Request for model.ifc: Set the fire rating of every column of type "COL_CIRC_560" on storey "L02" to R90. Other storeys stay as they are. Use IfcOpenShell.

First a look at what the model holds.

```python
import ifcopenshell
import ifcopenshell.util.element

model = ifcopenshell.open("model.ifc")
print(model.schema)
storey = next(s for s in model.by_type("IfcBuildingStorey") if s.Name == "L02")
columns = [e for e in ifcopenshell.util.element.get_decomposition(storey) if e.is_a("IfcColumn")]
seen = {}
for e in columns:
    element_type = ifcopenshell.util.element.get_type(e)
    key = (element_type.Name if element_type != e and element_type else None, ifcopenshell.util.element.get_pset(e, "Pset_ColumnCommon", "FireRating"))
    seen[key] = seen.get(key, 0) + 1
for (name, value), count in sorted(seen.items(), key=str):
    print(count, "x", name, "|", value)
```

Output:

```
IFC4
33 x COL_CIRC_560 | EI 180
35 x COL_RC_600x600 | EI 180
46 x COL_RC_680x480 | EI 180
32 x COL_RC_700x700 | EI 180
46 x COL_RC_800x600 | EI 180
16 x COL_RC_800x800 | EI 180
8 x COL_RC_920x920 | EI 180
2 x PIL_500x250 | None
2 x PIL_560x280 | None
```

```python
import ifcopenshell
import ifcopenshell.api.pset
import ifcopenshell.util.element

model = ifcopenshell.open("model.ifc")

storey = next(s for s in model.by_type("IfcBuildingStorey") if s.Name == "L02")
columns = [e for e in ifcopenshell.util.element.get_decomposition(storey) if e.is_a("IfcColumn")]

count = 0
for e in columns:
    element_type = ifcopenshell.util.element.get_type(e)
    if element_type in (None, e) or element_type.Name != "COL_CIRC_560":
        continue
    # add_pset returns the element's existing set when there is one.
    pset = ifcopenshell.api.pset.add_pset(model, product=e, name="Pset_ColumnCommon")
    ifcopenshell.api.pset.edit_pset(model, pset=pset, properties={"FireRating": "R90"})
    count += 1

print(count, "columns updated")

model.write("model_v2.ifc")
```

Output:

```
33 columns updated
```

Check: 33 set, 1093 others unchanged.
